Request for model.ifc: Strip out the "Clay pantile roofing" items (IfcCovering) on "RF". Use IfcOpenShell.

First a look at what the model holds.

```python
import ifcopenshell
import ifcopenshell.util.element

model = ifcopenshell.open("model.ifc")
print(model.schema)
storey = next(s for s in model.by_type("IfcBuildingStorey") if s.Name == "RF")
coverings = [e for e in ifcopenshell.util.element.get_decomposition(storey) if e.is_a("IfcCovering")]
seen = {}
for e in coverings:
    element_type = ifcopenshell.util.element.get_type(e)
    name = element_type.Name if element_type not in (None, e) else None
    seen[name] = seen.get(name, 0) + 1
for name, count in sorted(seen.items(), key=str):
    print(count, "x", name)
```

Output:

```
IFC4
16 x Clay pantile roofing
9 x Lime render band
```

```python
import ifcopenshell
import ifcopenshell.api.root
import ifcopenshell.util.element

model = ifcopenshell.open("model.ifc")

storey = next(s for s in model.by_type("IfcBuildingStorey") if s.Name == "RF")
coverings = [e for e in ifcopenshell.util.element.get_decomposition(storey) if e.is_a("IfcCovering")]
targets = [e for e in coverings if (t := ifcopenshell.util.element.get_type(e)) not in (None, e) and t.Name == "Clay pantile roofing"]

for e in targets:
    ifcopenshell.api.root.remove_product(model, product=e)
print(len(targets), "removed")

model.write("model_rev.ifc")
```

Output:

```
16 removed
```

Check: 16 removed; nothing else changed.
